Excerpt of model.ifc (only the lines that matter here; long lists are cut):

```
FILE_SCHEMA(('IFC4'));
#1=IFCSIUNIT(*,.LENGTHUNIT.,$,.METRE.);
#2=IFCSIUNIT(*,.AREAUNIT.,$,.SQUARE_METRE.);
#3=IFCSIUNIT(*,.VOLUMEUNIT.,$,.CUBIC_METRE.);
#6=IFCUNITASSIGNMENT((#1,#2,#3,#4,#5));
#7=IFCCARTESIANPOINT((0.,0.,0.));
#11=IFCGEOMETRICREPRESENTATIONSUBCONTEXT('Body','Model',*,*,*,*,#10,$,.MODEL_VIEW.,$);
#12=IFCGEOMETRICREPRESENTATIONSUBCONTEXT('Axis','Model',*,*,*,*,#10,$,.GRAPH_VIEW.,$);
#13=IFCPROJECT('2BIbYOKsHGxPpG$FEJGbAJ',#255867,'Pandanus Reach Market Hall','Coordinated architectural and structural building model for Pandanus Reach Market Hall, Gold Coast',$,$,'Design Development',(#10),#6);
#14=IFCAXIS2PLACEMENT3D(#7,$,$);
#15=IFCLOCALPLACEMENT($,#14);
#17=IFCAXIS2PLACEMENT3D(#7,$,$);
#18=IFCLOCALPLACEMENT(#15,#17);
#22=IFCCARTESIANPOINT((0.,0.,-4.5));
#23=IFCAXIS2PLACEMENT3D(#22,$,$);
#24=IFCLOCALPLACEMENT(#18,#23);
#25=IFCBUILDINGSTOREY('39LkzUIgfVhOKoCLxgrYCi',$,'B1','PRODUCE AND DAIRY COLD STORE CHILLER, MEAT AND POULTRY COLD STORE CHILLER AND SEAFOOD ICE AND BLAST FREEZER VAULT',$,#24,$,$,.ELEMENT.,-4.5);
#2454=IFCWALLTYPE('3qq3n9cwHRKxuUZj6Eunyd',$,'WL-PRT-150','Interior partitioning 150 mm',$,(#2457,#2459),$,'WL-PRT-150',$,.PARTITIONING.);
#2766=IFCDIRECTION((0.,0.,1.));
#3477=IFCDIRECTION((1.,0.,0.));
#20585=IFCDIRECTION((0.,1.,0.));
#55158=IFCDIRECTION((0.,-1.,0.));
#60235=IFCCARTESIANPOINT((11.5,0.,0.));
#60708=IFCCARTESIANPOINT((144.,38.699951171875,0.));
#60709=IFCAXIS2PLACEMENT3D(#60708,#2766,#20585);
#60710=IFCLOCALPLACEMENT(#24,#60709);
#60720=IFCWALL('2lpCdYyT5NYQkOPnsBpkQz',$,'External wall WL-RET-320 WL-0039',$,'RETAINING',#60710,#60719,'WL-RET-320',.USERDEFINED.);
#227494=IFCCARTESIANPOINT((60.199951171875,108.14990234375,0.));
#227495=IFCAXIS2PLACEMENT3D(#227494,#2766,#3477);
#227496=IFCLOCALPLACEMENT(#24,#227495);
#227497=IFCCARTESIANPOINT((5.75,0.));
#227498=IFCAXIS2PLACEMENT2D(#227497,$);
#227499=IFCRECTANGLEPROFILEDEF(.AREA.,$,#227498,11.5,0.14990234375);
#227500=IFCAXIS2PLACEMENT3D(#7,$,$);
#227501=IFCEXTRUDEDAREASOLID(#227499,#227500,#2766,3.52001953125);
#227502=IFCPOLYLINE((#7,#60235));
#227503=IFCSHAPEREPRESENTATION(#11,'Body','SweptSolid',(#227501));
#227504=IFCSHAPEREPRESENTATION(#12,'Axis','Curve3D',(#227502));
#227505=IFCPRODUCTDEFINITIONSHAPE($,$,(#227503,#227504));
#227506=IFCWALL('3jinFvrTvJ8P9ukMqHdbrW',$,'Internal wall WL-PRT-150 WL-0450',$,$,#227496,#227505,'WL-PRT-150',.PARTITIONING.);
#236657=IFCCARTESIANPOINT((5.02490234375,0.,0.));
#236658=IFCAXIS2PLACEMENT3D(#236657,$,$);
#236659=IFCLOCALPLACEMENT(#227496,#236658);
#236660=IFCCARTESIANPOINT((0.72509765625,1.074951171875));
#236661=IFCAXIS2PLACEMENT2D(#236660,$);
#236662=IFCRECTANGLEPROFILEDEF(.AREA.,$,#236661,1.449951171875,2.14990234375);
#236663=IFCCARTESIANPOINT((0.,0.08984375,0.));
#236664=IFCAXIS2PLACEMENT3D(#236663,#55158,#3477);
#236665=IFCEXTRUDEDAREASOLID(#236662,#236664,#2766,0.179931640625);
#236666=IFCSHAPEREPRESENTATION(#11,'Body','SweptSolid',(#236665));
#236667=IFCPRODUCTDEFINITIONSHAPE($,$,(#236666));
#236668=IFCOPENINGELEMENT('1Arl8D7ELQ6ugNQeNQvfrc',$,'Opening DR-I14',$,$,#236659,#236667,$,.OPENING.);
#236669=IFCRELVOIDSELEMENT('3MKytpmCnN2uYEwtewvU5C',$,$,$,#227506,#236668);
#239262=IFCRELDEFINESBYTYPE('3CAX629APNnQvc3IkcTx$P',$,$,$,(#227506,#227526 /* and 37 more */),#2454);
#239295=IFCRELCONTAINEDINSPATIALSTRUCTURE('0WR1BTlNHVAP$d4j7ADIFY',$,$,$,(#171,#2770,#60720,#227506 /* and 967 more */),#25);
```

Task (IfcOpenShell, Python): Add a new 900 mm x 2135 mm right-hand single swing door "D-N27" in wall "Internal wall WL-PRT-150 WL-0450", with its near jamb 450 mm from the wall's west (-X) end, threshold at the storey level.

```python
import numpy as np
import ifcopenshell
import ifcopenshell.api.feature
import ifcopenshell.api.geometry
import ifcopenshell.api.root
import ifcopenshell.api.spatial
import ifcopenshell.geom
import ifcopenshell.util.element
import ifcopenshell.util.placement
import ifcopenshell.util.representation
import ifcopenshell.util.shape
import ifcopenshell.util.unit

model = ifcopenshell.open("model.ifc")
unit_scale = ifcopenshell.util.unit.calculate_unit_scale(model)
settings = ifcopenshell.geom.settings()


def volume(element):
    """Net volume in cubic metres, openings subtracted."""
    shape = ifcopenshell.geom.create_shape(settings, element)
    return ifcopenshell.util.shape.get_volume(shape.geometry)


wall = model.by_id(227506)
storey = ifcopenshell.util.element.get_container(wall, ifc_class="IfcBuildingStorey")
context = ifcopenshell.util.representation.get_context(model, "Model", "Body", "MODEL_VIEW")
before = volume(wall)

width, height, from_end, sill = 0.9, 2.135, 0.45, 0.0  # metres

# The wall runs along its own X axis, and the end named is its -X end.
wall_shape = ifcopenshell.geom.create_shape(settings, wall)
x, y, z = ifcopenshell.util.shape.get_vertices(wall_shape.geometry).T
start = x.min() + from_end
face, thickness = float(y.min()), float(y.max() - y.min())
wall_matrix = ifcopenshell.util.placement.get_local_placement(wall.ObjectPlacement)
level = ifcopenshell.util.placement.get_local_placement(storey.ObjectPlacement)[2, 3]


def in_wall(x, y):
    """Placement at x, y metres in the wall's axes, at sill height."""
    matrix = wall_matrix.copy()
    matrix[:, 3] = wall_matrix @ np.array([x / unit_scale, y / unit_scale, 0.0, 1.0])
    matrix[2, 3] = level + sill / unit_scale
    return matrix


# Opening: a box that overshoots both wall faces by 50 mm.
opening = ifcopenshell.api.root.create_entity(model, ifc_class="IfcOpeningElement", predefined_type="OPENING")
box = ifcopenshell.api.geometry.add_wall_representation(
    model, context=context, length=width, height=height, thickness=thickness + 0.1
)
ifcopenshell.api.geometry.assign_representation(model, product=opening, representation=box)
ifcopenshell.api.geometry.edit_object_placement(model, product=opening, matrix=in_wall(start, face - 0.05), is_si=False)
ifcopenshell.api.feature.add_feature(model, feature=opening, element=wall)

door = ifcopenshell.api.root.create_entity(model, ifc_class="IfcDoor", name="D-N27", predefined_type="DOOR")
door.OverallWidth, door.OverallHeight = width / unit_scale, height / unit_scale
door.OperationType = "SINGLE_SWING_RIGHT"
body = ifcopenshell.api.geometry.add_door_representation(
    model,
    context=context,
    overall_width=door.OverallWidth,
    overall_height=door.OverallHeight,
    operation_type="SINGLE_SWING_RIGHT",
    lining_properties={"LiningDepth": thickness / unit_scale, "ThresholdDepth": thickness / unit_scale},
)
ifcopenshell.api.geometry.assign_representation(model, product=door, representation=body)
ifcopenshell.api.spatial.assign_container(model, products=[door], relating_structure=storey)
ifcopenshell.api.feature.add_filling(model, opening=opening, element=door)

# The lining spans the wall, so the door starts at the wall face.
ifcopenshell.api.geometry.edit_object_placement(model, product=door, matrix=in_wall(start, face), is_si=False)

after = volume(wall)

print(f"wall volume {before:.3f} -> {after:.3f} m3")

model.write("model_updated.ifc")
```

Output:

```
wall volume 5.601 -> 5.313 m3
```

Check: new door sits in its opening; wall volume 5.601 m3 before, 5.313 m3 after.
